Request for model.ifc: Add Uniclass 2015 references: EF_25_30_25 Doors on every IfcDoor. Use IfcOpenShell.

First a look at what the model holds.

```python
import ifcopenshell

model = ifcopenshell.open("model.ifc")
print(model.schema)
print("classifications:", [c.Name for c in model.by_type("IfcClassification")])
for ifc_class in ("IfcDoor", "IfcRoof", "IfcStair", "IfcWall", "IfcWindow"):
    print(ifc_class, len(model.by_type(ifc_class)))
```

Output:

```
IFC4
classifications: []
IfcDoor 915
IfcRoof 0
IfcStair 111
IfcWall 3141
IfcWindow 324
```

```python
import ifcopenshell
import ifcopenshell.api.classification

model = ifcopenshell.open("model.ifc")

system = ifcopenshell.api.classification.add_classification(model, classification="Uniclass 2015")

codes = {
    "IfcDoor": ("EF_25_30_25", "Doors"),
}
for ifc_class, (code, name) in codes.items():
    products = model.by_type(ifc_class)
    ifcopenshell.api.classification.add_reference(
        model, products=products, classification=system, identification=code, name=name
    )
    print(code, len(products))

model.write("model-out.ifc")
```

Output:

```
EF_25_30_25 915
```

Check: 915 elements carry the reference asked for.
